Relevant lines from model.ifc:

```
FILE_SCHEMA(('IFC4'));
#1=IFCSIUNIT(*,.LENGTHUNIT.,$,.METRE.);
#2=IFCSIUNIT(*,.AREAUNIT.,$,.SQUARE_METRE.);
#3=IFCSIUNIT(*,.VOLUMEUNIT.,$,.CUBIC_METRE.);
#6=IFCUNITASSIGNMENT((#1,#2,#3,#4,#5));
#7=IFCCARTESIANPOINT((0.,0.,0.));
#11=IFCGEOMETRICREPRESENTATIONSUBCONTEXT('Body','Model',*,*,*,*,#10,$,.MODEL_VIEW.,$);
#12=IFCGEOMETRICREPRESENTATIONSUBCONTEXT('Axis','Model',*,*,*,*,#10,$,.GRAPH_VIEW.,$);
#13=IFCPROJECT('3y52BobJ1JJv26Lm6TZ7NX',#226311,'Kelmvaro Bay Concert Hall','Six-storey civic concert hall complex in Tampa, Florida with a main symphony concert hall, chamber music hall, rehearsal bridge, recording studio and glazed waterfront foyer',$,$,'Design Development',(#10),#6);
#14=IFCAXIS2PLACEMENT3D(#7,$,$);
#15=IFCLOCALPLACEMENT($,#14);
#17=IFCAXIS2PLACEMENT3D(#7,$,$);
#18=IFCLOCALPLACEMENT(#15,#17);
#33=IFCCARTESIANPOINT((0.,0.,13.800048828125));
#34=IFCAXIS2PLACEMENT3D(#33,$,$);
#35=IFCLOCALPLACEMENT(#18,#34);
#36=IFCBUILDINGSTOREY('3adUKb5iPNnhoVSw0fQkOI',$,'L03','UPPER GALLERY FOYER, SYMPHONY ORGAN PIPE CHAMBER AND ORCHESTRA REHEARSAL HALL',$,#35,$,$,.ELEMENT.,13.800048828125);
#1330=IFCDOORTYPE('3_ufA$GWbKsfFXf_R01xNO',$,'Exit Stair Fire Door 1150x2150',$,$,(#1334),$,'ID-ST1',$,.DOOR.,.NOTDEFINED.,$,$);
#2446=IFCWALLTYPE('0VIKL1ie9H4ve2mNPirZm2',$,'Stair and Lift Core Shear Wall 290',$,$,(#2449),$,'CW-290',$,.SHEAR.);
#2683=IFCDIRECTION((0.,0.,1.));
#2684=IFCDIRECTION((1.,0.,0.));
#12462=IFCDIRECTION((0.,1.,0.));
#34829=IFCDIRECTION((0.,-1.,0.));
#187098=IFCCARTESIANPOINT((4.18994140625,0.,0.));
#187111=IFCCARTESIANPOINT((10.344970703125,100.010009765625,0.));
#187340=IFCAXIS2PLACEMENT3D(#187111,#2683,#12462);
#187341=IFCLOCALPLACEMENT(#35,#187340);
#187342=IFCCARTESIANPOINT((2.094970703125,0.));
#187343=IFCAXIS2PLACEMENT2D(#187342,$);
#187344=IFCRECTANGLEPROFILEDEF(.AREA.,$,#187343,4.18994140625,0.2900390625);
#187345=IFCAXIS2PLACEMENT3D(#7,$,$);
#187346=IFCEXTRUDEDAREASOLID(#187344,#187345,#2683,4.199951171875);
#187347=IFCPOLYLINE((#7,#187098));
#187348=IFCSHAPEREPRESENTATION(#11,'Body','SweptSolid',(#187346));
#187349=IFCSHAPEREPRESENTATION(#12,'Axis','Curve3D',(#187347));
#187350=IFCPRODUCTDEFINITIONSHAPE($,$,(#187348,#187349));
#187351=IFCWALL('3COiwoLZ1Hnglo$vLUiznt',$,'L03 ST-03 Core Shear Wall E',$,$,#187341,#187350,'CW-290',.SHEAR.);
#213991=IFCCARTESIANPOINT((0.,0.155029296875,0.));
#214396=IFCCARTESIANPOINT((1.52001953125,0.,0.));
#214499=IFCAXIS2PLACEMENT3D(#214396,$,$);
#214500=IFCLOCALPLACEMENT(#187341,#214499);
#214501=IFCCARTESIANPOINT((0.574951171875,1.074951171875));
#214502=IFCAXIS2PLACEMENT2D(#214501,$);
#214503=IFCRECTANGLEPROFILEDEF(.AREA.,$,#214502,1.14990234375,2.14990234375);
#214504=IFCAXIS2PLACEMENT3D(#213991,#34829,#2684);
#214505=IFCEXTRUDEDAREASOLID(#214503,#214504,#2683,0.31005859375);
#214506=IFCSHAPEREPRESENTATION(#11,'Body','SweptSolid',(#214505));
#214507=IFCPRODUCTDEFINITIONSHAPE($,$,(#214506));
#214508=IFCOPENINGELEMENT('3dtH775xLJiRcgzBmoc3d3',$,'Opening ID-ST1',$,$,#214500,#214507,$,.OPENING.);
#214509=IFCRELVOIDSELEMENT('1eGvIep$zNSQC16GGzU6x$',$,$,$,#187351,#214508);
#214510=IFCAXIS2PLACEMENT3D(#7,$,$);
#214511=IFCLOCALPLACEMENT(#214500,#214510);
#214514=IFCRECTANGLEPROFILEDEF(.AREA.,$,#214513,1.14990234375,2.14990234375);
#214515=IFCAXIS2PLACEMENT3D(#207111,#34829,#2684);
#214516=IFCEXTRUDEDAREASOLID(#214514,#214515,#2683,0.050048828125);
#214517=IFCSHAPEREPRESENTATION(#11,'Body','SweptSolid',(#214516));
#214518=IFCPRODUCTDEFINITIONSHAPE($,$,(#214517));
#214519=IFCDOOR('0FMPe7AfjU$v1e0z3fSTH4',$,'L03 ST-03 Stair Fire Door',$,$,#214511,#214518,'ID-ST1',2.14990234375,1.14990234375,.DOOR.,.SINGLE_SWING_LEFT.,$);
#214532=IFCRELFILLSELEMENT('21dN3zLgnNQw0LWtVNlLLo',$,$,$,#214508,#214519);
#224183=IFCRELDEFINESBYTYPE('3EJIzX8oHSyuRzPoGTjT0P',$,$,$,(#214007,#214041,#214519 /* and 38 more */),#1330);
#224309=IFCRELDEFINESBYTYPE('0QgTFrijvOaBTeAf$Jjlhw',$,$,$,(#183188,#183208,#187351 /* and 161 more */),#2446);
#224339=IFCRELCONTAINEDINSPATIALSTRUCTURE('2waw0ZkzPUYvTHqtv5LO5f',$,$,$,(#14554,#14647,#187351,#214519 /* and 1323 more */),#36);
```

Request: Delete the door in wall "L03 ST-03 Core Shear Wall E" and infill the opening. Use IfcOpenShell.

```python
import ifcopenshell
import ifcopenshell.api.feature
import ifcopenshell.api.root
import ifcopenshell.geom
import ifcopenshell.util.shape

model = ifcopenshell.open("model.ifc")
settings = ifcopenshell.geom.settings()


def volume(element):
    """Net volume in cubic metres, openings subtracted."""
    shape = ifcopenshell.geom.create_shape(settings, element)
    return ifcopenshell.util.shape.get_volume(shape.geometry)


door = model.by_guid("0FMPe7AfjU$v1e0z3fSTH4")
opening = door.FillsVoids[0].RelatingOpeningElement
wall = opening.VoidsElements[0].RelatingBuildingElement
before = volume(wall)

ifcopenshell.api.root.remove_product(model, product=door)
ifcopenshell.api.feature.remove_feature(model, feature=opening)

after = volume(wall)

print(f"wall volume {before:.3f} -> {after:.3f} m3")

model.write("model_v2.ifc")
```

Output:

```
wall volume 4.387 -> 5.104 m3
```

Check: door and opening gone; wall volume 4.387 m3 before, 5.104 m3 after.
